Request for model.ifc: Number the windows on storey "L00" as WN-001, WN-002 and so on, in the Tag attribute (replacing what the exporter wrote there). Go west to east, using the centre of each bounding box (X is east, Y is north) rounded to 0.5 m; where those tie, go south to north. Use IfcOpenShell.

First a look at what the model holds.

```python
import ifcopenshell
import ifcopenshell.util.element
import ifcopenshell.util.placement

model = ifcopenshell.open("model.ifc")
print(model.schema)
storey = next(s for s in model.by_type("IfcBuildingStorey") if s.Name == "L00")
windows = [e for e in ifcopenshell.util.element.get_decomposition(storey) if e.is_a("IfcWindow")]
for e in sorted(windows, key=lambda e: e.id()):
    origin = ifcopenshell.util.placement.get_local_placement(e.ObjectPlacement)[:3, 3]
    print(e.id(), e.Tag, e.Name, origin.round(2) + 0.0, sep=" | ")
```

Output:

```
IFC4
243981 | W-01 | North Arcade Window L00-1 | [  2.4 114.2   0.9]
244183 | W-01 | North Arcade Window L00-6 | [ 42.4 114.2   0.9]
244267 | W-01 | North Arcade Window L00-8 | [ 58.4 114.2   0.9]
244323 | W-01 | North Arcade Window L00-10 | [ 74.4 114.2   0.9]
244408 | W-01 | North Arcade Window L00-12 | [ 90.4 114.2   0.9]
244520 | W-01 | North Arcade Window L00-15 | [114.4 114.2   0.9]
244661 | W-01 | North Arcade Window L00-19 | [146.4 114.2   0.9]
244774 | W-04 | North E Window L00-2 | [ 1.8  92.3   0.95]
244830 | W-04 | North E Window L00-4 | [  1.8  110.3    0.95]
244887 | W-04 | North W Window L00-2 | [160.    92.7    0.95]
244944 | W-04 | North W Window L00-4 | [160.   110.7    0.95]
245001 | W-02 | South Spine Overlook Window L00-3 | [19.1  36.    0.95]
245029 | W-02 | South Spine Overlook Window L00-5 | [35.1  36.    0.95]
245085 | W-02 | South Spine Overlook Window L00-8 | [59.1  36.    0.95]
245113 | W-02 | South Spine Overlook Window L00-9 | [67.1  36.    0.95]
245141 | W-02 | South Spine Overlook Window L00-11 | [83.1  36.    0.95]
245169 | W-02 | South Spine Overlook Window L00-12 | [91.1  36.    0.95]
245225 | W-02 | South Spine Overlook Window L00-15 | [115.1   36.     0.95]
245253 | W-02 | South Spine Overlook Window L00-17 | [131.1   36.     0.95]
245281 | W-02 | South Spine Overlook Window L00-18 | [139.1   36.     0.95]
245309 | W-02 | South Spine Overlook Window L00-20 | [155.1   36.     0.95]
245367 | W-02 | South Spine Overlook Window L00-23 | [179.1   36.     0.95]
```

```python
import ifcopenshell
import ifcopenshell.geom
import ifcopenshell.util.element
import ifcopenshell.util.shape

model = ifcopenshell.open("model.ifc")
settings = ifcopenshell.geom.settings()
settings.set("use-world-coords", True)


def centre(element):
    shape = ifcopenshell.geom.create_shape(settings, element)
    return ifcopenshell.util.shape.get_bbox_centroid(shape.geometry)


storey = next(s for s in model.by_type("IfcBuildingStorey") if s.Name == "L00")
windows = [e for e in ifcopenshell.util.element.get_decomposition(storey) if e.is_a("IfcWindow")]

# Insertion points can sit at a corner or the storey origin, so sort by the geometry (in metres).
centres = {e: centre(e) for e in windows}
windows.sort(key=lambda e: (round(centres[e][0] / 0.5), centres[e][1]))

for i, e in enumerate(windows, start=1):
    number = f"WN-0{i:02d}"
    e.Tag = number
    print(e.id(), number)

model.write("model-out.ifc")
```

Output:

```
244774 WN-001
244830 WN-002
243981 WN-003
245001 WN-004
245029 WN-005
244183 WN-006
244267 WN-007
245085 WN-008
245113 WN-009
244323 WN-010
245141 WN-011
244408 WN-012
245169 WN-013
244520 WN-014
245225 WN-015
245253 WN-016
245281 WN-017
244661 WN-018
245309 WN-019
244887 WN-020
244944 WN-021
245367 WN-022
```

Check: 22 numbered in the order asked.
